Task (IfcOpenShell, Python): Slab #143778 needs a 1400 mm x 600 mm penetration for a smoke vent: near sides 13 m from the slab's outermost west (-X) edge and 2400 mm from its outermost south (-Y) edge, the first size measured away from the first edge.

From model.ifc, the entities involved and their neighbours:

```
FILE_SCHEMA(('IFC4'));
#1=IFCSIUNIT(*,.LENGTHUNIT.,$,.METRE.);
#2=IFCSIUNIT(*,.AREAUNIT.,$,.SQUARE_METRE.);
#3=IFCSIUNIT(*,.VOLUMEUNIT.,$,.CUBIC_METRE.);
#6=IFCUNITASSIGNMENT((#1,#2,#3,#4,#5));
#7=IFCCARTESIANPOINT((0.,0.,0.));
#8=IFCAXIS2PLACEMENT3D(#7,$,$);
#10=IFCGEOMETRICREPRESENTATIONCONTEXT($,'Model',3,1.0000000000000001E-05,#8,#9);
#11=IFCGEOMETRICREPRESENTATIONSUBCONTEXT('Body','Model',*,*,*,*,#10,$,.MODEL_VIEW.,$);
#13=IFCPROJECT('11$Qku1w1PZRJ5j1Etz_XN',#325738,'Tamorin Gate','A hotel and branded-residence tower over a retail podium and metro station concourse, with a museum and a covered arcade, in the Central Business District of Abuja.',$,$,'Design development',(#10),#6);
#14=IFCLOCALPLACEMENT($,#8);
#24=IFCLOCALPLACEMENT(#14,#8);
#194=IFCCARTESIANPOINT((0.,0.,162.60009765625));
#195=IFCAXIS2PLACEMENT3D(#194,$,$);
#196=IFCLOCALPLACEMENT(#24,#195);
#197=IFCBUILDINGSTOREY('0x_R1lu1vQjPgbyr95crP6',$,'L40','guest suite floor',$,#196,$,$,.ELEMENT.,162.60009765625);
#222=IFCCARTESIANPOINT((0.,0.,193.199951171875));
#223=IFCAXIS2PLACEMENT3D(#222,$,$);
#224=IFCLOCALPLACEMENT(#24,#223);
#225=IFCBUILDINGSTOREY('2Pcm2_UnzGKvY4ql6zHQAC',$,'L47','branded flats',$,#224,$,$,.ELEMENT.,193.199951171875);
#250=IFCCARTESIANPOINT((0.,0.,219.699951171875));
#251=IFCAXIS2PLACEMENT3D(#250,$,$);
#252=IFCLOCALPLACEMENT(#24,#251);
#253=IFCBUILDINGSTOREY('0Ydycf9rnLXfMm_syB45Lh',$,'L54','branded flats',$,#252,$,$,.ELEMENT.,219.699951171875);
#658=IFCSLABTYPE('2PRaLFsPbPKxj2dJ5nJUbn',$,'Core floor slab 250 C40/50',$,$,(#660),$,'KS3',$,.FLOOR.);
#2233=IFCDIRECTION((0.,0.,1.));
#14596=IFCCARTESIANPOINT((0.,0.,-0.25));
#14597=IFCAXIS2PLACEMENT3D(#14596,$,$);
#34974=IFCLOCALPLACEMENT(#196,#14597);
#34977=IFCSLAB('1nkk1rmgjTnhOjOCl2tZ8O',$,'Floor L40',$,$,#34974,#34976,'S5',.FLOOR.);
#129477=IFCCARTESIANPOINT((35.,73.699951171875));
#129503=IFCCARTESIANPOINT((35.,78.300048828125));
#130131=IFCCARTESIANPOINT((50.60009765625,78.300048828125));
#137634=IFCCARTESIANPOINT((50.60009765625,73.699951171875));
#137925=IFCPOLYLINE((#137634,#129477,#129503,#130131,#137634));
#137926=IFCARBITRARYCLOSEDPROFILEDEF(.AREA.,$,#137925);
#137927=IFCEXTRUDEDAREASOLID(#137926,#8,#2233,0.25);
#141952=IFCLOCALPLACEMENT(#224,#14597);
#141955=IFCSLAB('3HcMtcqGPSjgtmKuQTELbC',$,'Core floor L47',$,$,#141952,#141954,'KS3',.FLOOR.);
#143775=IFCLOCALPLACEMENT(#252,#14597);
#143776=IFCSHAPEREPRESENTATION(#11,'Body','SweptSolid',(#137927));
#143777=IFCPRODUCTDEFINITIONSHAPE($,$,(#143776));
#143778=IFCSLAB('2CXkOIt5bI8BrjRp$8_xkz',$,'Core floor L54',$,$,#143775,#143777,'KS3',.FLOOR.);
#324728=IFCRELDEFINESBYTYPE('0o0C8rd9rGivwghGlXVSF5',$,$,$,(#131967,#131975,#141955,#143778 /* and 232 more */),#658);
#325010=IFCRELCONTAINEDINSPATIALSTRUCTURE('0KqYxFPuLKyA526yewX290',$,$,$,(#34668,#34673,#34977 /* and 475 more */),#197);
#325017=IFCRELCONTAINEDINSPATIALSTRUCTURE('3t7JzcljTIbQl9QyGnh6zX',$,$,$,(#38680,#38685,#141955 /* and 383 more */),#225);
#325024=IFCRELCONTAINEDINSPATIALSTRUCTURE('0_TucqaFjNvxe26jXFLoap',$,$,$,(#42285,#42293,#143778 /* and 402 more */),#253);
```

```python
import numpy as np
import ifcopenshell
import ifcopenshell.api.feature
import ifcopenshell.api.geometry
import ifcopenshell.api.root
import ifcopenshell.geom
import ifcopenshell.util.placement
import ifcopenshell.util.representation
import ifcopenshell.util.shape
import ifcopenshell.util.unit

model = ifcopenshell.open("model.ifc")
unit_scale = ifcopenshell.util.unit.calculate_unit_scale(model)
settings = ifcopenshell.geom.settings()


def volume(element):
    """Net volume in cubic metres, openings subtracted."""
    shape = ifcopenshell.geom.create_shape(settings, element)
    return ifcopenshell.util.shape.get_volume(shape.geometry)


slab = model.by_guid("2CXkOIt5bI8BrjRp$8_xkz")
before = volume(slab)

# Extent in the slab's own axes, in metres. The edges named are its -X and -Y sides.
slab_shape = ifcopenshell.geom.create_shape(settings, slab)
vertices = ifcopenshell.util.shape.get_vertices(slab_shape.geometry)
x_min, y_min, bottom = vertices.min(axis=0)
top = vertices[:, 2].max()

opening = ifcopenshell.api.root.create_entity(model, ifc_class="IfcOpeningElement", name="Smoke vent opening", predefined_type="OPENING")
context = ifcopenshell.util.representation.get_context(model, "Model", "Body", "MODEL_VIEW")
width, depth = 1.4, 0.6
outline = [(0.0, 0.0), (width, 0.0), (width, depth), (0.0, depth), (0.0, 0.0)]
# Overshoot both faces by 50 mm so the cut is clean.
shape = ifcopenshell.api.geometry.add_slab_representation(
    model, context=context, depth=top - bottom + 0.1, polyline=outline
)
ifcopenshell.api.geometry.assign_representation(model, product=opening, representation=shape)

matrix = ifcopenshell.util.placement.get_local_placement(slab.ObjectPlacement)
matrix[:, 3] = matrix @ np.append(np.array([x_min + 13, y_min + 2.4, bottom - 0.05]) / unit_scale, 1.0)
ifcopenshell.api.geometry.edit_object_placement(model, product=opening, matrix=matrix, is_si=False)
ifcopenshell.api.feature.add_feature(model, feature=opening, element=slab)

after = volume(slab)

print(f"slab volume {before:.3f} -> {after:.3f} m3")

model.write("model_v2.ifc")
```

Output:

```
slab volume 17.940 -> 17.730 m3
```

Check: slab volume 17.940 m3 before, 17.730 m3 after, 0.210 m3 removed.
